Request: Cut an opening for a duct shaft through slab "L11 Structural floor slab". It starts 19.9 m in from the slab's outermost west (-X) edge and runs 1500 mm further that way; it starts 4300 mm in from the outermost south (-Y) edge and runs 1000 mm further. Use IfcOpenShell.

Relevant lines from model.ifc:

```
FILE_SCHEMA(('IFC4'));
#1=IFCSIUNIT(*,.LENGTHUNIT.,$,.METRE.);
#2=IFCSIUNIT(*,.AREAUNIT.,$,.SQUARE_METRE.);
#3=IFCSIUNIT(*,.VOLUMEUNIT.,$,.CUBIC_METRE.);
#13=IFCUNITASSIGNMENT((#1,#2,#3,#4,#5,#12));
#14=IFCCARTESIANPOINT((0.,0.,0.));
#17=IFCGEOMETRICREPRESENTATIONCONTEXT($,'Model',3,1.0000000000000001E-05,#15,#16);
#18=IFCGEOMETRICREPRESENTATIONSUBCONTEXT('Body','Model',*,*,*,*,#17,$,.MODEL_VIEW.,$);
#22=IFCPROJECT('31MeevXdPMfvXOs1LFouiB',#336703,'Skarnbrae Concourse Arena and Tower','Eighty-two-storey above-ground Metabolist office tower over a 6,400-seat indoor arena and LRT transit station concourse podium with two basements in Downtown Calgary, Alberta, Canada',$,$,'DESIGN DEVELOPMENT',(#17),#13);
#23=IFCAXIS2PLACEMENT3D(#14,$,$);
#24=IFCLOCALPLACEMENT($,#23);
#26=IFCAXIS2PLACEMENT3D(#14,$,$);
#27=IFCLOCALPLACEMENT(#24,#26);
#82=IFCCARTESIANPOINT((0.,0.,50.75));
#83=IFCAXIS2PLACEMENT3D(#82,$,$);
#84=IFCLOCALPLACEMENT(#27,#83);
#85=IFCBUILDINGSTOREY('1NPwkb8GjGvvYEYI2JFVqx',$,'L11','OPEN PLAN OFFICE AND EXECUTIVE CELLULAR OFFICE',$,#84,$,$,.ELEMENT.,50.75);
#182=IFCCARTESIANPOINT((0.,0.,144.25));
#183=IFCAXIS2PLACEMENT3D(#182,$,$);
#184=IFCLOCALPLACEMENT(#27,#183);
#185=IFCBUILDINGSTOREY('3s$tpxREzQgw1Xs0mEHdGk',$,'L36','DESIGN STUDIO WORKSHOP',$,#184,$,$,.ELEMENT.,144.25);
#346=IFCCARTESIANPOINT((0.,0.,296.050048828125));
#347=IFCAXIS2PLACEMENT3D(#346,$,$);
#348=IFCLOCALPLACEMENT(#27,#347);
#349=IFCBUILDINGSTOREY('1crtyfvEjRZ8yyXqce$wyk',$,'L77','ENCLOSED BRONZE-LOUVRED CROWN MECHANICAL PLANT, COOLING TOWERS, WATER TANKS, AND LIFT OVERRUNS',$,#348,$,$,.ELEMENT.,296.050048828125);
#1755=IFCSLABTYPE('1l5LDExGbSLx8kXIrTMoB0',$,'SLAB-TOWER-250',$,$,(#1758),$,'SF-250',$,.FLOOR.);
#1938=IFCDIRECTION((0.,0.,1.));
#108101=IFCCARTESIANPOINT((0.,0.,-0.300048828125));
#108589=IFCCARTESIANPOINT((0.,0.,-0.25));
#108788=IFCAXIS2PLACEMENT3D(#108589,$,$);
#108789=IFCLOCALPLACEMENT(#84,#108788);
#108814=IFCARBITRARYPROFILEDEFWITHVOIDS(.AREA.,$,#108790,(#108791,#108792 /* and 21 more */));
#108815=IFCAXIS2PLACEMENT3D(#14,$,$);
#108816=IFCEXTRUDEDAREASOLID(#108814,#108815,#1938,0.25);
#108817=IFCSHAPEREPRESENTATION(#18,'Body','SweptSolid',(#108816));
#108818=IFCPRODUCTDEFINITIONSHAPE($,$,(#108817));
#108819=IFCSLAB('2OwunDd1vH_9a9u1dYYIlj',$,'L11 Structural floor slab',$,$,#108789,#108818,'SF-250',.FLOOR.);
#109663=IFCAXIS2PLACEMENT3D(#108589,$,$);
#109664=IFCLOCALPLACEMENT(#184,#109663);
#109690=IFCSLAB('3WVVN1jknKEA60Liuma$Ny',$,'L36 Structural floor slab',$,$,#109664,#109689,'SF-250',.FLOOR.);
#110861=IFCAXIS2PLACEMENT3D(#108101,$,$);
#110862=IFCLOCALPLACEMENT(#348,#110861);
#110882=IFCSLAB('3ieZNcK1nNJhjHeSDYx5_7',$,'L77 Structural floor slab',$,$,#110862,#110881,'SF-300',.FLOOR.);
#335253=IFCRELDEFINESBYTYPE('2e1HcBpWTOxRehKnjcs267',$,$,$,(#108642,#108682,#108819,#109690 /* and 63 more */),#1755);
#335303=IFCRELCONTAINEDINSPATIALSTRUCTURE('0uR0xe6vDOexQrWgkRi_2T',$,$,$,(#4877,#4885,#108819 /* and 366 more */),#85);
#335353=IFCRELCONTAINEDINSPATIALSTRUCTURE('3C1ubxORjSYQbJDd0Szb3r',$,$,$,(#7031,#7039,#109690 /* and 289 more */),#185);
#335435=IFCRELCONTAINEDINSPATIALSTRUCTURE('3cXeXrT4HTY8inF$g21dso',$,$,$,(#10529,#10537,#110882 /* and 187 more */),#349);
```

```python
import numpy as np
import ifcopenshell
import ifcopenshell.api.feature
import ifcopenshell.api.geometry
import ifcopenshell.api.root
import ifcopenshell.geom
import ifcopenshell.util.placement
import ifcopenshell.util.representation
import ifcopenshell.util.shape
import ifcopenshell.util.unit

model = ifcopenshell.open("model.ifc")
unit_scale = ifcopenshell.util.unit.calculate_unit_scale(model)
settings = ifcopenshell.geom.settings()


def volume(element):
    """Net volume in cubic metres, openings subtracted."""
    shape = ifcopenshell.geom.create_shape(settings, element)
    return ifcopenshell.util.shape.get_volume(shape.geometry)


slab = model.by_guid("2OwunDd1vH_9a9u1dYYIlj")
before = volume(slab)

# Extent in the slab's own axes, in metres. The edges named are its -X and -Y sides.
slab_shape = ifcopenshell.geom.create_shape(settings, slab)
vertices = ifcopenshell.util.shape.get_vertices(slab_shape.geometry)
x_min, y_min, bottom = vertices.min(axis=0)
top = vertices[:, 2].max()

opening = ifcopenshell.api.root.create_entity(model, ifc_class="IfcOpeningElement", name="Duct shaft opening", predefined_type="OPENING")
context = ifcopenshell.util.representation.get_context(model, "Model", "Body", "MODEL_VIEW")
width, depth = 1.5, 1
outline = [(0.0, 0.0), (width, 0.0), (width, depth), (0.0, depth), (0.0, 0.0)]
# Overshoot both faces by 50 mm so the cut is clean.
shape = ifcopenshell.api.geometry.add_slab_representation(
    model, context=context, depth=top - bottom + 0.1, polyline=outline
)
ifcopenshell.api.geometry.assign_representation(model, product=opening, representation=shape)

matrix = ifcopenshell.util.placement.get_local_placement(slab.ObjectPlacement)
matrix[:, 3] = matrix @ np.append(np.array([x_min + 19.9, y_min + 4.3, bottom - 0.05]) / unit_scale, 1.0)
ifcopenshell.api.geometry.edit_object_placement(model, product=opening, matrix=matrix, is_si=False)
ifcopenshell.api.feature.add_feature(model, feature=opening, element=slab)

after = volume(slab)

print(f"slab volume {before:.3f} -> {after:.3f} m3")

model.write("model_updated.ifc")
```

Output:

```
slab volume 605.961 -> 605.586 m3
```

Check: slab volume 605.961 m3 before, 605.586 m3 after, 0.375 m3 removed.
